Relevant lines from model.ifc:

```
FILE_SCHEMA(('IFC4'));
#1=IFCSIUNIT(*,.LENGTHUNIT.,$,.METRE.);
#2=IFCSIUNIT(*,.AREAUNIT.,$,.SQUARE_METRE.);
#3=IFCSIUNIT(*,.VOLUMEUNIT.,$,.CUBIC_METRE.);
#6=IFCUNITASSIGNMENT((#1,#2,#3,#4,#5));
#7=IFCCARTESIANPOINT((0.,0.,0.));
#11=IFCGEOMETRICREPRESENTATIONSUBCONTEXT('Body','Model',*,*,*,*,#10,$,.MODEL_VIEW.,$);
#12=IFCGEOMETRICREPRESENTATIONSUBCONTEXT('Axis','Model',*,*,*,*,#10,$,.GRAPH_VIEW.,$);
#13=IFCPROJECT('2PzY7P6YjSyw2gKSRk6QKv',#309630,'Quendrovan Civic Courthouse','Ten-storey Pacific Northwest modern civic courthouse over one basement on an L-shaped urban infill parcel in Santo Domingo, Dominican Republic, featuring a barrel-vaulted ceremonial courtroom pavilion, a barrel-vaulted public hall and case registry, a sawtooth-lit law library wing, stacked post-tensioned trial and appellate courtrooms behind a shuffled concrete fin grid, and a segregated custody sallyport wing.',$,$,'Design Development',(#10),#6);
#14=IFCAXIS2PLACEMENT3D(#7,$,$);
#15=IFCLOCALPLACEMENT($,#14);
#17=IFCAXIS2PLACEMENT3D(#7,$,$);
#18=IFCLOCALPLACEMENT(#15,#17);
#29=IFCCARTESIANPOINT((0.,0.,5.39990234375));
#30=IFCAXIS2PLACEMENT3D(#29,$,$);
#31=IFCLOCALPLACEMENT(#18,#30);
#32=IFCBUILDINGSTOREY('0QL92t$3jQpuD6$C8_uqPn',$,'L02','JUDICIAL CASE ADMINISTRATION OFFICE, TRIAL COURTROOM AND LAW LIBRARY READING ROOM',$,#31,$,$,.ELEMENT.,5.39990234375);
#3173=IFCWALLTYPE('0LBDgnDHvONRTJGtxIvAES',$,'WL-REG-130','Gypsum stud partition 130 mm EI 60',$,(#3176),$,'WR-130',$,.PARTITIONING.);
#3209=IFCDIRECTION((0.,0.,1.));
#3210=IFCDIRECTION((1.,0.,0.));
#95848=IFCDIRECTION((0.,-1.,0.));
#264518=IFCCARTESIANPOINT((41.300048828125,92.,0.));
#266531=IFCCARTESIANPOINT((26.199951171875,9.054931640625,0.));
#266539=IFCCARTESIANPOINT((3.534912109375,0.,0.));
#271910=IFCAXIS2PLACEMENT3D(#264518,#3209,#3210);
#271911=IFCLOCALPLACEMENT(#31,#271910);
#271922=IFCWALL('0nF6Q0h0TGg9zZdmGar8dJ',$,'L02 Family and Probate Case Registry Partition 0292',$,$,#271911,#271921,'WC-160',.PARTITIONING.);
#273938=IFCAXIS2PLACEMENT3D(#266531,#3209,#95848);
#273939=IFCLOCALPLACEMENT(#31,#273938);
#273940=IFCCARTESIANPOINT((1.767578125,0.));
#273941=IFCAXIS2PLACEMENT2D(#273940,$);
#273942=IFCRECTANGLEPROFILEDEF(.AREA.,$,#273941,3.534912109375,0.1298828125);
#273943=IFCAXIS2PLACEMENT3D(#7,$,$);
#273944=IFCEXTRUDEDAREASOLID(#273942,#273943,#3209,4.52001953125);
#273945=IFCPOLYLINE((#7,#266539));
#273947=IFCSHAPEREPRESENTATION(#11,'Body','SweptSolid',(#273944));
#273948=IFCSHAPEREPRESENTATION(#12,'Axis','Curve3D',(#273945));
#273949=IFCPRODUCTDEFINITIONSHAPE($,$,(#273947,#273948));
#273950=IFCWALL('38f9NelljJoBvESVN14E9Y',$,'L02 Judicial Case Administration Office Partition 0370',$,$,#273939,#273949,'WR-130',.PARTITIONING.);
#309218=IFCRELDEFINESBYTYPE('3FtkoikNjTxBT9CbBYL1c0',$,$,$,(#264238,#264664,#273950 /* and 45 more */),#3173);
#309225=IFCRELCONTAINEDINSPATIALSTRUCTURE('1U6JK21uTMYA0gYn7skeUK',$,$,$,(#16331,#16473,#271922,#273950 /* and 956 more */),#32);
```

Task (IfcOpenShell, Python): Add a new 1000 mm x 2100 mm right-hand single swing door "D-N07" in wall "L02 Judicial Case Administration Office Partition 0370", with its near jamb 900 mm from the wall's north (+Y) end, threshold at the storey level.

```python
import numpy as np
import ifcopenshell
import ifcopenshell.api.feature
import ifcopenshell.api.geometry
import ifcopenshell.api.root
import ifcopenshell.api.spatial
import ifcopenshell.geom
import ifcopenshell.util.element
import ifcopenshell.util.placement
import ifcopenshell.util.representation
import ifcopenshell.util.shape
import ifcopenshell.util.unit

model = ifcopenshell.open("model.ifc")
unit_scale = ifcopenshell.util.unit.calculate_unit_scale(model)
settings = ifcopenshell.geom.settings()


def volume(element):
    """Net volume in cubic metres, openings subtracted."""
    shape = ifcopenshell.geom.create_shape(settings, element)
    return ifcopenshell.util.shape.get_volume(shape.geometry)


wall = model.by_id(273950)
storey = ifcopenshell.util.element.get_container(wall, ifc_class="IfcBuildingStorey")
context = ifcopenshell.util.representation.get_context(model, "Model", "Body", "MODEL_VIEW")
before = volume(wall)

width, height, from_end, sill = 1, 2.1, 0.9, 0.0  # metres

# The wall runs along its own X axis, and the end named is its -X end.
wall_shape = ifcopenshell.geom.create_shape(settings, wall)
x, y, z = ifcopenshell.util.shape.get_vertices(wall_shape.geometry).T
start = x.min() + from_end
face, thickness = float(y.min()), float(y.max() - y.min())
wall_matrix = ifcopenshell.util.placement.get_local_placement(wall.ObjectPlacement)
level = ifcopenshell.util.placement.get_local_placement(storey.ObjectPlacement)[2, 3]


def in_wall(x, y):
    """Placement at x, y metres in the wall's axes, at sill height."""
    matrix = wall_matrix.copy()
    matrix[:, 3] = wall_matrix @ np.array([x / unit_scale, y / unit_scale, 0.0, 1.0])
    matrix[2, 3] = level + sill / unit_scale
    return matrix


# Opening: a box that overshoots both wall faces by 50 mm.
opening = ifcopenshell.api.root.create_entity(model, ifc_class="IfcOpeningElement", predefined_type="OPENING")
box = ifcopenshell.api.geometry.add_wall_representation(
    model, context=context, length=width, height=height, thickness=thickness + 0.1
)
ifcopenshell.api.geometry.assign_representation(model, product=opening, representation=box)
ifcopenshell.api.geometry.edit_object_placement(model, product=opening, matrix=in_wall(start, face - 0.05), is_si=False)
ifcopenshell.api.feature.add_feature(model, feature=opening, element=wall)

door = ifcopenshell.api.root.create_entity(model, ifc_class="IfcDoor", name="D-N07", predefined_type="DOOR")
door.OverallWidth, door.OverallHeight = width / unit_scale, height / unit_scale
door.OperationType = "SINGLE_SWING_RIGHT"
body = ifcopenshell.api.geometry.add_door_representation(
    model,
    context=context,
    overall_width=door.OverallWidth,
    overall_height=door.OverallHeight,
    operation_type="SINGLE_SWING_RIGHT",
    lining_properties={"LiningDepth": thickness / unit_scale, "ThresholdDepth": thickness / unit_scale},
)
ifcopenshell.api.geometry.assign_representation(model, product=door, representation=body)
ifcopenshell.api.spatial.assign_container(model, products=[door], relating_structure=storey)
ifcopenshell.api.feature.add_filling(model, opening=opening, element=door)

# The lining spans the wall, so the door starts at the wall face.
ifcopenshell.api.geometry.edit_object_placement(model, product=door, matrix=in_wall(start, face), is_si=False)

after = volume(wall)

print(f"wall volume {before:.3f} -> {after:.3f} m3")

model.write("model_edited.ifc")
```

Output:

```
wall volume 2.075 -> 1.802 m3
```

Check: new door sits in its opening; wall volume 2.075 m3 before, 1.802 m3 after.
